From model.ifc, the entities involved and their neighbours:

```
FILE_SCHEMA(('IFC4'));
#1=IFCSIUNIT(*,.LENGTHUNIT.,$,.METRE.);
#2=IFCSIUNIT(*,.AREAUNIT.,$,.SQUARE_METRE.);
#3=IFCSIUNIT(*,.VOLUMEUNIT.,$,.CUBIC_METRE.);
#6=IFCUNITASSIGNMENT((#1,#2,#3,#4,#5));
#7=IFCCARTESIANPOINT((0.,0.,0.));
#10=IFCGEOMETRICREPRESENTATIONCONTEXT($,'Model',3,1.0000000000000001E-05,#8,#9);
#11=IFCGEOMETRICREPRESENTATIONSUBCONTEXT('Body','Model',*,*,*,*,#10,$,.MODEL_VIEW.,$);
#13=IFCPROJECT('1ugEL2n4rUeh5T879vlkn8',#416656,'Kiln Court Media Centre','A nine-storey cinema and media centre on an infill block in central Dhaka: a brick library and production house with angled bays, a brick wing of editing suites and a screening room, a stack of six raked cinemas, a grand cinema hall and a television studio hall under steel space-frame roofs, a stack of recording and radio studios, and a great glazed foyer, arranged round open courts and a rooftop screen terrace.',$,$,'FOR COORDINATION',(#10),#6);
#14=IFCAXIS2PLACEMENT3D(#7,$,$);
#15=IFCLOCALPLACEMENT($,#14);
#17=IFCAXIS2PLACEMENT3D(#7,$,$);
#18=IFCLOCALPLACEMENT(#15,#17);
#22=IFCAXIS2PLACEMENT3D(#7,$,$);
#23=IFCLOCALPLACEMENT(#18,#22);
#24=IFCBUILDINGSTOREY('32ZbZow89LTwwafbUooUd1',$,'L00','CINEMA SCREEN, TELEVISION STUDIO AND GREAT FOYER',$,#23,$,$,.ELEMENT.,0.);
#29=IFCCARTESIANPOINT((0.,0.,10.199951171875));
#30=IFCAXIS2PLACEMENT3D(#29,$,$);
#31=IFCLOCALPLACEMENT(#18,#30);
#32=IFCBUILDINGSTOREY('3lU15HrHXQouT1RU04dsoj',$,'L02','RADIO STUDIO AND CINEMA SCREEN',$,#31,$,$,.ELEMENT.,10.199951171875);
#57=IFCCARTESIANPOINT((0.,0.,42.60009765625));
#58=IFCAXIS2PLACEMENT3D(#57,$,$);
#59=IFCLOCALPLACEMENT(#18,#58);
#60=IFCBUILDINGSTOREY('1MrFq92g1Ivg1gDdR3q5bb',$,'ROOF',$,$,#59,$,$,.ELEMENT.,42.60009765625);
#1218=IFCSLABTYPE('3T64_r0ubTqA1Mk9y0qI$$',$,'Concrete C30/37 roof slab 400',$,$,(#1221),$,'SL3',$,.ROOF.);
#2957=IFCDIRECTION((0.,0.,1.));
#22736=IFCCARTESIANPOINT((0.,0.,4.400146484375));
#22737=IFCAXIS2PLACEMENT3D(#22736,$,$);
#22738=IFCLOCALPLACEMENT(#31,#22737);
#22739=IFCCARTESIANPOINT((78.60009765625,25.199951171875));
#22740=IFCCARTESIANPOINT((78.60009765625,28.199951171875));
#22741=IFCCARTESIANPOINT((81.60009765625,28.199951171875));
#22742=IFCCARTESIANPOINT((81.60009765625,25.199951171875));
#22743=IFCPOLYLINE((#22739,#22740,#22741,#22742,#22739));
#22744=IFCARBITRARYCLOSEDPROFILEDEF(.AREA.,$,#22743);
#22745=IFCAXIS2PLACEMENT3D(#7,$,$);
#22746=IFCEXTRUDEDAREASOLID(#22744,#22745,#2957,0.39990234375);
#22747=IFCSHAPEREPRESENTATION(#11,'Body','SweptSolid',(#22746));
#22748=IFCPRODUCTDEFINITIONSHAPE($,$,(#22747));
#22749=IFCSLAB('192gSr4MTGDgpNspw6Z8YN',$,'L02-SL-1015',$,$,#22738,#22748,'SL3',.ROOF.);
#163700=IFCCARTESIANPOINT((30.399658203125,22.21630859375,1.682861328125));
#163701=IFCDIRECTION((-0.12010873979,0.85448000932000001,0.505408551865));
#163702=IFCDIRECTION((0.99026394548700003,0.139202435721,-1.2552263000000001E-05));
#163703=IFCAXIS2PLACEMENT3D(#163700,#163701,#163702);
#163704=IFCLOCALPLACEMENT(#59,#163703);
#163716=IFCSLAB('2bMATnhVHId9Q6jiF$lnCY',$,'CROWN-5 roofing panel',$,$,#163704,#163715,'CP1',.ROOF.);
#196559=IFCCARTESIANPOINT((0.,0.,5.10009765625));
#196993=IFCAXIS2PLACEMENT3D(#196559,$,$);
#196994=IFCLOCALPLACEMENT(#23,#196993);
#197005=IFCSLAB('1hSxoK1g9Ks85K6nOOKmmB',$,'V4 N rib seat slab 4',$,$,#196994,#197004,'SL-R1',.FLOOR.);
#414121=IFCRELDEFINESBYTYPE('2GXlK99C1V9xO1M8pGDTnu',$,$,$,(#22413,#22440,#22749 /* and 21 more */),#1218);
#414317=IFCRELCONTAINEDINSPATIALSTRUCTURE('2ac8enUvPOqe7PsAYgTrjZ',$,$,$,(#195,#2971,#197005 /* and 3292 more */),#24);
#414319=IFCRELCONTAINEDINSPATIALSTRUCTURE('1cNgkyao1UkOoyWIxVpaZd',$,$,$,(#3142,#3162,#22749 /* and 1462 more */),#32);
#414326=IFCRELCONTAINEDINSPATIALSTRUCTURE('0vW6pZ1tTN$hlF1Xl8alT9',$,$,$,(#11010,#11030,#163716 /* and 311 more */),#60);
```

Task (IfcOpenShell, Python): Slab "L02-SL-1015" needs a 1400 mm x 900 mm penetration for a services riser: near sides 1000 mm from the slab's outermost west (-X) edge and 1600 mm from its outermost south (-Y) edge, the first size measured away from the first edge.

```python
import numpy as np
import ifcopenshell
import ifcopenshell.api.feature
import ifcopenshell.api.geometry
import ifcopenshell.api.root
import ifcopenshell.geom
import ifcopenshell.util.placement
import ifcopenshell.util.representation
import ifcopenshell.util.shape
import ifcopenshell.util.unit

model = ifcopenshell.open("model.ifc")
unit_scale = ifcopenshell.util.unit.calculate_unit_scale(model)
settings = ifcopenshell.geom.settings()


def volume(element):
    """Net volume in cubic metres, openings subtracted."""
    shape = ifcopenshell.geom.create_shape(settings, element)
    return ifcopenshell.util.shape.get_volume(shape.geometry)


slab = model.by_guid("192gSr4MTGDgpNspw6Z8YN")
before = volume(slab)

# Extent in the slab's own axes, in metres. The edges named are its -X and -Y sides.
slab_shape = ifcopenshell.geom.create_shape(settings, slab)
vertices = ifcopenshell.util.shape.get_vertices(slab_shape.geometry)
x_min, y_min, bottom = vertices.min(axis=0)
top = vertices[:, 2].max()

opening = ifcopenshell.api.root.create_entity(model, ifc_class="IfcOpeningElement", name="Services riser opening", predefined_type="OPENING")
context = ifcopenshell.util.representation.get_context(model, "Model", "Body", "MODEL_VIEW")
width, depth = 1.4, 0.9
outline = [(0.0, 0.0), (width, 0.0), (width, depth), (0.0, depth), (0.0, 0.0)]
# Overshoot both faces by 50 mm so the cut is clean.
shape = ifcopenshell.api.geometry.add_slab_representation(
    model, context=context, depth=top - bottom + 0.1, polyline=outline
)
ifcopenshell.api.geometry.assign_representation(model, product=opening, representation=shape)

matrix = ifcopenshell.util.placement.get_local_placement(slab.ObjectPlacement)
matrix[:, 3] = matrix @ np.append(np.array([x_min + 1, y_min + 1.6, bottom - 0.05]) / unit_scale, 1.0)
ifcopenshell.api.geometry.edit_object_placement(model, product=opening, matrix=matrix, is_si=False)
ifcopenshell.api.feature.add_feature(model, feature=opening, element=slab)

after = volume(slab)

print(f"slab volume {before:.3f} -> {after:.3f} m3")

model.write("model_edited.ifc")
```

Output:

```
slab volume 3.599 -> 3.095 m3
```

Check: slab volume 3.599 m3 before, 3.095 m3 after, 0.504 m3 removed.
